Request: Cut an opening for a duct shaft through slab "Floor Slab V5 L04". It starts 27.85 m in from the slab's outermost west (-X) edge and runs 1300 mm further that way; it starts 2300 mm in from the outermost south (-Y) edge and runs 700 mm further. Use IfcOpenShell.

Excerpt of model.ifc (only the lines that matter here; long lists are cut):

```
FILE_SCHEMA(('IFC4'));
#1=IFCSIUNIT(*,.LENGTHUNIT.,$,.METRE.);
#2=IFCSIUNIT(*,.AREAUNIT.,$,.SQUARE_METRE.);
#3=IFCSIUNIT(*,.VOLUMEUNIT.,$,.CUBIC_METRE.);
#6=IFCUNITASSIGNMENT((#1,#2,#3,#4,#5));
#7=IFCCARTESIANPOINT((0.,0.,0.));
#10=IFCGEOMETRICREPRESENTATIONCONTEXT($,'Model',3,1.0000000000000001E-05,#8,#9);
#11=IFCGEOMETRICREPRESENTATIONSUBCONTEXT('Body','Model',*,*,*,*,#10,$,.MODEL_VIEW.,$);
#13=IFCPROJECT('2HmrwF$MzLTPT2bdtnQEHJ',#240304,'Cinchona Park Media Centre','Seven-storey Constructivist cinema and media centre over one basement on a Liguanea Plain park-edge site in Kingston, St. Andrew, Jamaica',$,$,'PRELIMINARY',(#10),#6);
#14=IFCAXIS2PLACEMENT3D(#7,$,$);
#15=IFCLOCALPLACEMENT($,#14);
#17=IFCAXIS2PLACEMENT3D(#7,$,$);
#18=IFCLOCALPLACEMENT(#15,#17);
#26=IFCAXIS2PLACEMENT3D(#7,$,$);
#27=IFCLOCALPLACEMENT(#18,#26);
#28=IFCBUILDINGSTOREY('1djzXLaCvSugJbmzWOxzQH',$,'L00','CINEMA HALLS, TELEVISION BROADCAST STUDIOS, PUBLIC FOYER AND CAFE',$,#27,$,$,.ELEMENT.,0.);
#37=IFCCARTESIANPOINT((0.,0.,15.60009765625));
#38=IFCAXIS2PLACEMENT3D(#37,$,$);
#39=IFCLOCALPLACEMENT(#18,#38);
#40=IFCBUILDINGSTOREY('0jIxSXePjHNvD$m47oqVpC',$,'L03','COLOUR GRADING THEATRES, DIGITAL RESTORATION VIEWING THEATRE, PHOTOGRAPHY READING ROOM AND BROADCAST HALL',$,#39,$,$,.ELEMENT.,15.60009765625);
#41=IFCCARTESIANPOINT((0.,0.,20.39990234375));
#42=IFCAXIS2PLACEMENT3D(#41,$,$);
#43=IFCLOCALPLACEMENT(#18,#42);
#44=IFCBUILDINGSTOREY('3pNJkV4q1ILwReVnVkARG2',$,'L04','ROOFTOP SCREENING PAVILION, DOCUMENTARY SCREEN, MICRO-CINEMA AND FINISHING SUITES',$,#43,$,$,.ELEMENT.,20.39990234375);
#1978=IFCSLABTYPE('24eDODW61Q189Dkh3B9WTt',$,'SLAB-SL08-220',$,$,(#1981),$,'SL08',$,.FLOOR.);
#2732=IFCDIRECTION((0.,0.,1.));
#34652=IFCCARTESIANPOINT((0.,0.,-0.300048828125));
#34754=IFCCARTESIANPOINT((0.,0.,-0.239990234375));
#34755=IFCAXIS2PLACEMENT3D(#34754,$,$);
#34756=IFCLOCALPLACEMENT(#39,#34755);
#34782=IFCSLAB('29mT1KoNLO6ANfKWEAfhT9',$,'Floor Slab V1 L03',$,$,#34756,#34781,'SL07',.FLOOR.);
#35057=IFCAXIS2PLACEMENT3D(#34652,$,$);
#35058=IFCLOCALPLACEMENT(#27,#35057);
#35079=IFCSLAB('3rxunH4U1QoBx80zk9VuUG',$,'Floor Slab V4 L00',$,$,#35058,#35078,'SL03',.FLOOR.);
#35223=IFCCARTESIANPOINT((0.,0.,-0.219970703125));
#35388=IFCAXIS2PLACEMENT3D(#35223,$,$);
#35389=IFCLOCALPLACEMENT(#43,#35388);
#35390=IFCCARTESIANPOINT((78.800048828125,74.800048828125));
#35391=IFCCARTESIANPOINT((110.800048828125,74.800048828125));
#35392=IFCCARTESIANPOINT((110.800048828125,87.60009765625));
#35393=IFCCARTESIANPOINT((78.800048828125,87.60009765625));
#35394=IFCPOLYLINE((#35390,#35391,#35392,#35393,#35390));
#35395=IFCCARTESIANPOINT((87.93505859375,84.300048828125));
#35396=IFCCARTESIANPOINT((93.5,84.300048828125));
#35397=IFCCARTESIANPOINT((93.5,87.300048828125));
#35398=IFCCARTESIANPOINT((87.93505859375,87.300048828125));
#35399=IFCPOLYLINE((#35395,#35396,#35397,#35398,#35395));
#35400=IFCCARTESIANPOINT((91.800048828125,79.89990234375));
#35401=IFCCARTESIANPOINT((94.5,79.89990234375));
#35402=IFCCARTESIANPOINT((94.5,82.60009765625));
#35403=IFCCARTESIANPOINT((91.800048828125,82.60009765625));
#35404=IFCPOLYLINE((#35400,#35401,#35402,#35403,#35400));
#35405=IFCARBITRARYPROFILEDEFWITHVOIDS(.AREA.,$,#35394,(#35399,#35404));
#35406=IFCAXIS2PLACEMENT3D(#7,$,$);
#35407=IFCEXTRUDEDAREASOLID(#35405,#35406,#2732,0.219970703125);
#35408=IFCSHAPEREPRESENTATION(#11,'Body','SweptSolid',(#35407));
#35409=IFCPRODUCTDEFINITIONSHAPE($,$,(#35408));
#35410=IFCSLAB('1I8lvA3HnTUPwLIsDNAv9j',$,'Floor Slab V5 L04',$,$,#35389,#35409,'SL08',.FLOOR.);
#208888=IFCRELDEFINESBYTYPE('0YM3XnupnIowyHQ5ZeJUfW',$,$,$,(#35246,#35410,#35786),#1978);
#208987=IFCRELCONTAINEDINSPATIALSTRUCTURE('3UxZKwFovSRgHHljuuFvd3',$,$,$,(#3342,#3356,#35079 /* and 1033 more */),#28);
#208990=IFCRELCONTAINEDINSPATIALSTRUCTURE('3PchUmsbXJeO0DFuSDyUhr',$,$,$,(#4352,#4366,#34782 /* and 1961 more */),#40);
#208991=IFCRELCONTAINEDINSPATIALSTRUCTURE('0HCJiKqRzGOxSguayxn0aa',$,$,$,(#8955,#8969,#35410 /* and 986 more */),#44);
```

```python
import numpy as np
import ifcopenshell
import ifcopenshell.api.feature
import ifcopenshell.api.geometry
import ifcopenshell.api.root
import ifcopenshell.geom
import ifcopenshell.util.placement
import ifcopenshell.util.representation
import ifcopenshell.util.shape
import ifcopenshell.util.unit

model = ifcopenshell.open("model.ifc")
unit_scale = ifcopenshell.util.unit.calculate_unit_scale(model)
settings = ifcopenshell.geom.settings()


def volume(element):
    """Net volume in cubic metres, openings subtracted."""
    shape = ifcopenshell.geom.create_shape(settings, element)
    return ifcopenshell.util.shape.get_volume(shape.geometry)


slab = model.by_id(35410)
before = volume(slab)

# Extent in the slab's own axes, in metres. The edges named are its -X and -Y sides.
slab_shape = ifcopenshell.geom.create_shape(settings, slab)
vertices = ifcopenshell.util.shape.get_vertices(slab_shape.geometry)
x_min, y_min, bottom = vertices.min(axis=0)
top = vertices[:, 2].max()

opening = ifcopenshell.api.root.create_entity(model, ifc_class="IfcOpeningElement", name="Duct shaft opening", predefined_type="OPENING")
context = ifcopenshell.util.representation.get_context(model, "Model", "Body", "MODEL_VIEW")
width, depth = 1.3, 0.7
outline = [(0.0, 0.0), (width, 0.0), (width, depth), (0.0, depth), (0.0, 0.0)]
# Overshoot both faces by 50 mm so the cut is clean.
shape = ifcopenshell.api.geometry.add_slab_representation(
    model, context=context, depth=top - bottom + 0.1, polyline=outline
)
ifcopenshell.api.geometry.assign_representation(model, product=opening, representation=shape)

matrix = ifcopenshell.util.placement.get_local_placement(slab.ObjectPlacement)
matrix[:, 3] = matrix @ np.append(np.array([x_min + 27.85, y_min + 2.3, bottom - 0.05]) / unit_scale, 1.0)
ifcopenshell.api.geometry.edit_object_placement(model, product=opening, matrix=matrix, is_si=False)
ifcopenshell.api.feature.add_feature(model, feature=opening, element=slab)

after = volume(slab)

print(f"slab volume {before:.3f} -> {after:.3f} m3")

model.write("model_v2.ifc")
```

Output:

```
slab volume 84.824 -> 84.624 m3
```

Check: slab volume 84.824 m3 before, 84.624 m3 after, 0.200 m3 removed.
